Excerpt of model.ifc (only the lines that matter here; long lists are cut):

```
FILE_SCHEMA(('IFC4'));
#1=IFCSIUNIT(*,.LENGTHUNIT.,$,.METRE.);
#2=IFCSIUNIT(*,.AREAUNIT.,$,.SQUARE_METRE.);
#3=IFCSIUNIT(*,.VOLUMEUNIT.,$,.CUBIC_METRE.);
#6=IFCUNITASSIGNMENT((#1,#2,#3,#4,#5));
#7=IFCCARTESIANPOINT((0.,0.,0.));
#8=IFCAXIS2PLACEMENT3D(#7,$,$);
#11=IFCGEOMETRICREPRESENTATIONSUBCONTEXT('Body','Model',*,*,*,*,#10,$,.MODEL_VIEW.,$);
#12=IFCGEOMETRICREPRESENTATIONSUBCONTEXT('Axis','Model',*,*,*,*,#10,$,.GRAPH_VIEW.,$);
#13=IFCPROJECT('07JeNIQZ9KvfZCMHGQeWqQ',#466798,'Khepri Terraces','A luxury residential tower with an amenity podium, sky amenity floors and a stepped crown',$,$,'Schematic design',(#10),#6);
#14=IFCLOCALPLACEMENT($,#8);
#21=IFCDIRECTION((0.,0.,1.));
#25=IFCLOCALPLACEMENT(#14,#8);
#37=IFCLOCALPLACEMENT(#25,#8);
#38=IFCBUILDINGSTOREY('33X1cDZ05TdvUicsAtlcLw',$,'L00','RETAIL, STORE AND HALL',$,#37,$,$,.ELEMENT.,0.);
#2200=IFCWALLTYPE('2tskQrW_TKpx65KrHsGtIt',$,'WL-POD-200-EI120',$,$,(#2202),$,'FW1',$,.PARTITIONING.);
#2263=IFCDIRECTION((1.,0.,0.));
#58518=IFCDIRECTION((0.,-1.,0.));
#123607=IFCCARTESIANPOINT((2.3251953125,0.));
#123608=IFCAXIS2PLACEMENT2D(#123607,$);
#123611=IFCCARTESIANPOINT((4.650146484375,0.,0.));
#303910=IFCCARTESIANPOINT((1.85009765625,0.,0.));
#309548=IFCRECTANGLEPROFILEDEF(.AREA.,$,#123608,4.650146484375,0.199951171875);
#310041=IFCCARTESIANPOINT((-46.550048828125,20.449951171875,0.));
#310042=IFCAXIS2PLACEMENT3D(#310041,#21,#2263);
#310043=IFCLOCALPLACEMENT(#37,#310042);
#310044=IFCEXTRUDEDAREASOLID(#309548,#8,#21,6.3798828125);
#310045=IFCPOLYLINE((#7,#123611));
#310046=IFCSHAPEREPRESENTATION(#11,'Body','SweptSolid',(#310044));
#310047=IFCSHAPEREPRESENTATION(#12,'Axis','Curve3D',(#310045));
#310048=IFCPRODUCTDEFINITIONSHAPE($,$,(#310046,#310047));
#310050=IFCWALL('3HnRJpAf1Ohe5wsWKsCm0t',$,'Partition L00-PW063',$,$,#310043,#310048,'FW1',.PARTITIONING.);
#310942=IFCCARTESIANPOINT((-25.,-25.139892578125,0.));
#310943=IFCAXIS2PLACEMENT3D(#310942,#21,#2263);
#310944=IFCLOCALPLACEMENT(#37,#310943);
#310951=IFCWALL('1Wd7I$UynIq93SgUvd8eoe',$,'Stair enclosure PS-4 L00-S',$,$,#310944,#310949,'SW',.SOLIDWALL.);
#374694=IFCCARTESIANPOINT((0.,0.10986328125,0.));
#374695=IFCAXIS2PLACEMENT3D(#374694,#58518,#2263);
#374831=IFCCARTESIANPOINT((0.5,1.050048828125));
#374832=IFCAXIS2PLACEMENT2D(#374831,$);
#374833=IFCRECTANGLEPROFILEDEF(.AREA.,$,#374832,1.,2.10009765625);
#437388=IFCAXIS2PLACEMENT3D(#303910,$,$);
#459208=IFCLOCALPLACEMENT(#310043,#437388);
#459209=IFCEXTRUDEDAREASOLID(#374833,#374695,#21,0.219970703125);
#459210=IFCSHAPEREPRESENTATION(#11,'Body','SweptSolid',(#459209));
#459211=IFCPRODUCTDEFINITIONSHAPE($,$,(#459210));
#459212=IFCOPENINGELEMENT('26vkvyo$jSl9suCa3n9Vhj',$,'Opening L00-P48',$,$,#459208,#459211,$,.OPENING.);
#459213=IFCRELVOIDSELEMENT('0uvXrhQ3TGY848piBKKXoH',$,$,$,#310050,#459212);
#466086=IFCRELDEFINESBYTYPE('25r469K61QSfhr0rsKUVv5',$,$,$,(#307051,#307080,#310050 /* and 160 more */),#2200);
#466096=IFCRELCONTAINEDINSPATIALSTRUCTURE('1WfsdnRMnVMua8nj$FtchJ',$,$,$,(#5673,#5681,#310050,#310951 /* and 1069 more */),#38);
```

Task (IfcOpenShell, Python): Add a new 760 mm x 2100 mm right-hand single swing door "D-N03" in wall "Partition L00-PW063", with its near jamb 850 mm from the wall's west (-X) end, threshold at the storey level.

```python
import numpy as np
import ifcopenshell
import ifcopenshell.api.feature
import ifcopenshell.api.geometry
import ifcopenshell.api.root
import ifcopenshell.api.spatial
import ifcopenshell.geom
import ifcopenshell.util.element
import ifcopenshell.util.placement
import ifcopenshell.util.representation
import ifcopenshell.util.shape
import ifcopenshell.util.unit

model = ifcopenshell.open("model.ifc")
unit_scale = ifcopenshell.util.unit.calculate_unit_scale(model)
settings = ifcopenshell.geom.settings()


def volume(element):
    """Net volume in cubic metres, openings subtracted."""
    shape = ifcopenshell.geom.create_shape(settings, element)
    return ifcopenshell.util.shape.get_volume(shape.geometry)


wall = model.by_id(310050)
storey = ifcopenshell.util.element.get_container(wall, ifc_class="IfcBuildingStorey")
context = ifcopenshell.util.representation.get_context(model, "Model", "Body", "MODEL_VIEW")
before = volume(wall)

width, height, from_end, sill = 0.76, 2.1, 0.85, 0.0  # metres

# The wall runs along its own X axis, and the end named is its -X end.
wall_shape = ifcopenshell.geom.create_shape(settings, wall)
x, y, z = ifcopenshell.util.shape.get_vertices(wall_shape.geometry).T
start = x.min() + from_end
face, thickness = float(y.min()), float(y.max() - y.min())
wall_matrix = ifcopenshell.util.placement.get_local_placement(wall.ObjectPlacement)
level = ifcopenshell.util.placement.get_local_placement(storey.ObjectPlacement)[2, 3]


def in_wall(x, y):
    """Placement at x, y metres in the wall's axes, at sill height."""
    matrix = wall_matrix.copy()
    matrix[:, 3] = wall_matrix @ np.array([x / unit_scale, y / unit_scale, 0.0, 1.0])
    matrix[2, 3] = level + sill / unit_scale
    return matrix


# Opening: a box that overshoots both wall faces by 50 mm.
opening = ifcopenshell.api.root.create_entity(model, ifc_class="IfcOpeningElement", predefined_type="OPENING")
box = ifcopenshell.api.geometry.add_wall_representation(
    model, context=context, length=width, height=height, thickness=thickness + 0.1
)
ifcopenshell.api.geometry.assign_representation(model, product=opening, representation=box)
ifcopenshell.api.geometry.edit_object_placement(model, product=opening, matrix=in_wall(start, face - 0.05), is_si=False)
ifcopenshell.api.feature.add_feature(model, feature=opening, element=wall)

door = ifcopenshell.api.root.create_entity(model, ifc_class="IfcDoor", name="D-N03", predefined_type="DOOR")
door.OverallWidth, door.OverallHeight = width / unit_scale, height / unit_scale
door.OperationType = "SINGLE_SWING_RIGHT"
body = ifcopenshell.api.geometry.add_door_representation(
    model,
    context=context,
    overall_width=door.OverallWidth,
    overall_height=door.OverallHeight,
    operation_type="SINGLE_SWING_RIGHT",
    lining_properties={"LiningDepth": thickness / unit_scale, "ThresholdDepth": thickness / unit_scale},
)
ifcopenshell.api.geometry.assign_representation(model, product=door, representation=body)
ifcopenshell.api.spatial.assign_container(model, products=[door], relating_structure=storey)
ifcopenshell.api.feature.add_filling(model, opening=opening, element=door)

# The lining spans the wall, so the door starts at the wall face.
ifcopenshell.api.geometry.edit_object_placement(model, product=door, matrix=in_wall(start, face), is_si=False)

after = volume(wall)

print(f"wall volume {before:.3f} -> {after:.3f} m3")

model.write("model_rev.ifc")
```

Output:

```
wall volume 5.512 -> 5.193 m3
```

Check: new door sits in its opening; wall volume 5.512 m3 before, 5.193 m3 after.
